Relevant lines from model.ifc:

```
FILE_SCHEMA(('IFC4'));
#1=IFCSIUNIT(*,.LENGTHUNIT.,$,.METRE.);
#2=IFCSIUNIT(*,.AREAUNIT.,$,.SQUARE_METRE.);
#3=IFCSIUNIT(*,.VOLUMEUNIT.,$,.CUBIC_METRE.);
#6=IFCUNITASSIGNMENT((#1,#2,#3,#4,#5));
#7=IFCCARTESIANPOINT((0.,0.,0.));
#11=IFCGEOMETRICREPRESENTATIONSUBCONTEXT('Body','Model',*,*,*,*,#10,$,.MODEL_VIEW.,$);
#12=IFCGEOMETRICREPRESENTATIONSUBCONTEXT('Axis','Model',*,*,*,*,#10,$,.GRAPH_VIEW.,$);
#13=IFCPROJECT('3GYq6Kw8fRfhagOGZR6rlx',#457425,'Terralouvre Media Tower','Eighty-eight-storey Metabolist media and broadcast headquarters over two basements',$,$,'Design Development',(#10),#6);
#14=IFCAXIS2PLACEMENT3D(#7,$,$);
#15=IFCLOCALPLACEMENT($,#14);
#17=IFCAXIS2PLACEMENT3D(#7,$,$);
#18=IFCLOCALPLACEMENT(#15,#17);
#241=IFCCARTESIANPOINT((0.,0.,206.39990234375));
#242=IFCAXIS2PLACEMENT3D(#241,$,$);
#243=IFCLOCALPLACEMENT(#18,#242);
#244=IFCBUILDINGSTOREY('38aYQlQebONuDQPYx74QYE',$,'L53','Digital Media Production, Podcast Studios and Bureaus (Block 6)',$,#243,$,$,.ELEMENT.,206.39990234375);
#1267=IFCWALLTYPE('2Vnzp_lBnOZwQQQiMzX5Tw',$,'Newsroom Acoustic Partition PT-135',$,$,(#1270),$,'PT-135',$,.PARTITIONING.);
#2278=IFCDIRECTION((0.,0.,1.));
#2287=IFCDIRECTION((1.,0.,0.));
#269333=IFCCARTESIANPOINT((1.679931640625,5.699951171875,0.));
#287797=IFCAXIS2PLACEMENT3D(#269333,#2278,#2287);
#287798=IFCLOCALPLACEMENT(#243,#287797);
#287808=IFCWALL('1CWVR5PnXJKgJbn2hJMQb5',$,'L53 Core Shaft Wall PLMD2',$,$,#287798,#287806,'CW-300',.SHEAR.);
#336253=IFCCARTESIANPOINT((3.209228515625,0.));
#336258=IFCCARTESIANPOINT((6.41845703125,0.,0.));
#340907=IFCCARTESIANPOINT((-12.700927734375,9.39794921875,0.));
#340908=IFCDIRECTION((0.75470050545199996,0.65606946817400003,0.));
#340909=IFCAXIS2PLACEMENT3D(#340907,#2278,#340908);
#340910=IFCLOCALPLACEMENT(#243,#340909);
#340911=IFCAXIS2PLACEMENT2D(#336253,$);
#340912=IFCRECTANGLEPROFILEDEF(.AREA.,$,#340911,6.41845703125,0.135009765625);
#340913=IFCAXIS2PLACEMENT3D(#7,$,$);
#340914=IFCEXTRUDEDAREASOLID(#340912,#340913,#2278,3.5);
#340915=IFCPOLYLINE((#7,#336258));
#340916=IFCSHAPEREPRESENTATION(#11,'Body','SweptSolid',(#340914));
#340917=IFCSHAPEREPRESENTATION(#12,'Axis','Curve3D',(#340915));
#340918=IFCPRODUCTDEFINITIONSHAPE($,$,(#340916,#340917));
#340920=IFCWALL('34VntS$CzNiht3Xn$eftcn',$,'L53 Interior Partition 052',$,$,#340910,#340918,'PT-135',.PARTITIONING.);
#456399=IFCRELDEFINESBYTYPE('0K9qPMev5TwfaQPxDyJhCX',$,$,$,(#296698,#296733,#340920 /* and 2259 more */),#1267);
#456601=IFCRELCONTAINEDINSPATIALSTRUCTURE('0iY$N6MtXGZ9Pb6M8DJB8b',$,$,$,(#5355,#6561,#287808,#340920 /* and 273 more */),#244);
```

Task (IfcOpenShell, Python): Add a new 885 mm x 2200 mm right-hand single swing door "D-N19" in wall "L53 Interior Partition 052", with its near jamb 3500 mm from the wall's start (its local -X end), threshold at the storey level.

```python
import numpy as np
import ifcopenshell
import ifcopenshell.api.feature
import ifcopenshell.api.geometry
import ifcopenshell.api.root
import ifcopenshell.api.spatial
import ifcopenshell.geom
import ifcopenshell.util.element
import ifcopenshell.util.placement
import ifcopenshell.util.representation
import ifcopenshell.util.shape
import ifcopenshell.util.unit

model = ifcopenshell.open("model.ifc")
unit_scale = ifcopenshell.util.unit.calculate_unit_scale(model)
settings = ifcopenshell.geom.settings()


def volume(element):
    """Net volume in cubic metres, openings subtracted."""
    shape = ifcopenshell.geom.create_shape(settings, element)
    return ifcopenshell.util.shape.get_volume(shape.geometry)


wall = model.by_guid("34VntS$CzNiht3Xn$eftcn")
storey = ifcopenshell.util.element.get_container(wall, ifc_class="IfcBuildingStorey")
context = ifcopenshell.util.representation.get_context(model, "Model", "Body", "MODEL_VIEW")
before = volume(wall)

width, height, from_end, sill = 0.885, 2.2, 3.5, 0.0  # metres

# The wall runs along its own X axis, and the end named is its -X end.
wall_shape = ifcopenshell.geom.create_shape(settings, wall)
x, y, z = ifcopenshell.util.shape.get_vertices(wall_shape.geometry).T
start = x.min() + from_end
face, thickness = float(y.min()), float(y.max() - y.min())
wall_matrix = ifcopenshell.util.placement.get_local_placement(wall.ObjectPlacement)
level = ifcopenshell.util.placement.get_local_placement(storey.ObjectPlacement)[2, 3]


def in_wall(x, y):
    """Placement at x, y metres in the wall's axes, at sill height."""
    matrix = wall_matrix.copy()
    matrix[:, 3] = wall_matrix @ np.array([x / unit_scale, y / unit_scale, 0.0, 1.0])
    matrix[2, 3] = level + sill / unit_scale
    return matrix


# Opening: a box that overshoots both wall faces by 50 mm.
opening = ifcopenshell.api.root.create_entity(model, ifc_class="IfcOpeningElement", predefined_type="OPENING")
box = ifcopenshell.api.geometry.add_wall_representation(
    model, context=context, length=width, height=height, thickness=thickness + 0.1
)
ifcopenshell.api.geometry.assign_representation(model, product=opening, representation=box)
ifcopenshell.api.geometry.edit_object_placement(model, product=opening, matrix=in_wall(start, face - 0.05), is_si=False)
ifcopenshell.api.feature.add_feature(model, feature=opening, element=wall)

door = ifcopenshell.api.root.create_entity(model, ifc_class="IfcDoor", name="D-N19", predefined_type="DOOR")
door.OverallWidth, door.OverallHeight = width / unit_scale, height / unit_scale
door.OperationType = "SINGLE_SWING_RIGHT"
body = ifcopenshell.api.geometry.add_door_representation(
    model,
    context=context,
    overall_width=door.OverallWidth,
    overall_height=door.OverallHeight,
    operation_type="SINGLE_SWING_RIGHT",
    lining_properties={"LiningDepth": thickness / unit_scale, "ThresholdDepth": thickness / unit_scale},
)
ifcopenshell.api.geometry.assign_representation(model, product=door, representation=body)
ifcopenshell.api.spatial.assign_container(model, products=[door], relating_structure=storey)
ifcopenshell.api.feature.add_filling(model, opening=opening, element=door)

# The lining spans the wall, so the door starts at the wall face.
ifcopenshell.api.geometry.edit_object_placement(model, product=door, matrix=in_wall(start, face), is_si=False)

after = volume(wall)

print(f"wall volume {before:.3f} -> {after:.3f} m3")

model.write("model-out.ifc")
```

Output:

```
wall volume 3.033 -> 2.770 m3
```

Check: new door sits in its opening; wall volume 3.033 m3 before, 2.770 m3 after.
